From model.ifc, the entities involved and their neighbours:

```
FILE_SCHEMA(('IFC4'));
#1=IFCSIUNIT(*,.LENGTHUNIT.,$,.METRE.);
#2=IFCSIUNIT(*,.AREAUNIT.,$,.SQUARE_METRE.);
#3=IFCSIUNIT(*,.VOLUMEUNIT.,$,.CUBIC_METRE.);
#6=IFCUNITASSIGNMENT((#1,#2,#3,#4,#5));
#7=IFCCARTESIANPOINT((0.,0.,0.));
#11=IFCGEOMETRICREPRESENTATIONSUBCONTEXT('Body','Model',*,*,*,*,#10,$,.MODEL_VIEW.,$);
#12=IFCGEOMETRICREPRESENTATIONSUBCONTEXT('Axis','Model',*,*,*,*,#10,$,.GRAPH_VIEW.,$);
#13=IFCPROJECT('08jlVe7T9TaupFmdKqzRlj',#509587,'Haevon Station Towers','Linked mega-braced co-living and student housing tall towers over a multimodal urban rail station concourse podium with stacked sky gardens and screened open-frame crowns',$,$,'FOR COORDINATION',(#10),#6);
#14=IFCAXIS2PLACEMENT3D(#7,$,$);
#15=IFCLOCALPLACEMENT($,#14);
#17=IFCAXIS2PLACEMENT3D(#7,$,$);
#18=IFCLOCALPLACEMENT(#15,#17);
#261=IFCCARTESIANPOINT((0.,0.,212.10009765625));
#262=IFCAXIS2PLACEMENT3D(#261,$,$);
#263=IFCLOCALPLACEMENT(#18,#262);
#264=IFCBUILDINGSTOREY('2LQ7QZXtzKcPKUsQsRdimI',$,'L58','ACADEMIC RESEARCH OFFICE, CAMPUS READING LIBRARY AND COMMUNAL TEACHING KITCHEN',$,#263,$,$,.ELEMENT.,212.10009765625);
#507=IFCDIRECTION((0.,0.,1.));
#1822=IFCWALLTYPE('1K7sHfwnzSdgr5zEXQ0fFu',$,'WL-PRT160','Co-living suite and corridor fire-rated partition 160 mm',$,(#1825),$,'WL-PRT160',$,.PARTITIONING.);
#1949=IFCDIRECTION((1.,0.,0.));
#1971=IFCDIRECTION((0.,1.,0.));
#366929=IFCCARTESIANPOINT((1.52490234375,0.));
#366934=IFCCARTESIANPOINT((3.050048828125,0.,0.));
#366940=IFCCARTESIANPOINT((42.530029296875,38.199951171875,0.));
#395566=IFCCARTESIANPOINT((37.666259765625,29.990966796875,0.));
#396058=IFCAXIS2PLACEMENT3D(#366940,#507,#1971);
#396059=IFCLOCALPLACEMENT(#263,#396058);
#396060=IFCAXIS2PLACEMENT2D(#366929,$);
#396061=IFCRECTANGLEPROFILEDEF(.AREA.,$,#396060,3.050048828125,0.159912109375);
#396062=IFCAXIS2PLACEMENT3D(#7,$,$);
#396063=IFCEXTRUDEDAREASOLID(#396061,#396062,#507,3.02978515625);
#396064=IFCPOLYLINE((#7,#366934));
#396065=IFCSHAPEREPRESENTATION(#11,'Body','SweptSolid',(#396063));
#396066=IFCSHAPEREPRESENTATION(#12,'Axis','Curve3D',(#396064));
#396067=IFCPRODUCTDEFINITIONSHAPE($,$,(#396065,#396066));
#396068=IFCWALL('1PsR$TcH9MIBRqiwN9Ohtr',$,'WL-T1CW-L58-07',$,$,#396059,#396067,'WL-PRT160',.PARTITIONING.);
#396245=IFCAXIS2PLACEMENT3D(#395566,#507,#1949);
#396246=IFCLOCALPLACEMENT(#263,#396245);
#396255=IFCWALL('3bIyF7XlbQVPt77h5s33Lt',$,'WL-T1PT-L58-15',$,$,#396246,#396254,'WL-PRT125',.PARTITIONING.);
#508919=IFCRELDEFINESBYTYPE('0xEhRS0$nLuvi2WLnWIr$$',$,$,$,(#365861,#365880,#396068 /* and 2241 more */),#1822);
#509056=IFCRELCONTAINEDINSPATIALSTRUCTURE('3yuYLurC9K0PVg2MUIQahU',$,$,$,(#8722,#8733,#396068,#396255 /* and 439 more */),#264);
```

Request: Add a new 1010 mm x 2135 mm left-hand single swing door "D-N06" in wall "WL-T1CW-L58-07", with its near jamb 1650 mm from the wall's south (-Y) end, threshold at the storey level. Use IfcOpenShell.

```python
import numpy as np
import ifcopenshell
import ifcopenshell.api.feature
import ifcopenshell.api.geometry
import ifcopenshell.api.root
import ifcopenshell.api.spatial
import ifcopenshell.geom
import ifcopenshell.util.element
import ifcopenshell.util.placement
import ifcopenshell.util.representation
import ifcopenshell.util.shape
import ifcopenshell.util.unit

model = ifcopenshell.open("model.ifc")
unit_scale = ifcopenshell.util.unit.calculate_unit_scale(model)
settings = ifcopenshell.geom.settings()


def volume(element):
    """Net volume in cubic metres, openings subtracted."""
    shape = ifcopenshell.geom.create_shape(settings, element)
    return ifcopenshell.util.shape.get_volume(shape.geometry)


wall = model.by_guid("1PsR$TcH9MIBRqiwN9Ohtr")
storey = ifcopenshell.util.element.get_container(wall, ifc_class="IfcBuildingStorey")
context = ifcopenshell.util.representation.get_context(model, "Model", "Body", "MODEL_VIEW")
before = volume(wall)

width, height, from_end, sill = 1.01, 2.135, 1.65, 0.0  # metres

# The wall runs along its own X axis, and the end named is its -X end.
wall_shape = ifcopenshell.geom.create_shape(settings, wall)
x, y, z = ifcopenshell.util.shape.get_vertices(wall_shape.geometry).T
start = x.min() + from_end
face, thickness = float(y.min()), float(y.max() - y.min())
wall_matrix = ifcopenshell.util.placement.get_local_placement(wall.ObjectPlacement)
level = ifcopenshell.util.placement.get_local_placement(storey.ObjectPlacement)[2, 3]


def in_wall(x, y):
    """Placement at x, y metres in the wall's axes, at sill height."""
    matrix = wall_matrix.copy()
    matrix[:, 3] = wall_matrix @ np.array([x / unit_scale, y / unit_scale, 0.0, 1.0])
    matrix[2, 3] = level + sill / unit_scale
    return matrix


# Opening: a box that overshoots both wall faces by 50 mm.
opening = ifcopenshell.api.root.create_entity(model, ifc_class="IfcOpeningElement", predefined_type="OPENING")
box = ifcopenshell.api.geometry.add_wall_representation(
    model, context=context, length=width, height=height, thickness=thickness + 0.1
)
ifcopenshell.api.geometry.assign_representation(model, product=opening, representation=box)
ifcopenshell.api.geometry.edit_object_placement(model, product=opening, matrix=in_wall(start, face - 0.05), is_si=False)
ifcopenshell.api.feature.add_feature(model, feature=opening, element=wall)

door = ifcopenshell.api.root.create_entity(model, ifc_class="IfcDoor", name="D-N06", predefined_type="DOOR")
door.OverallWidth, door.OverallHeight = width / unit_scale, height / unit_scale
door.OperationType = "SINGLE_SWING_LEFT"
body = ifcopenshell.api.geometry.add_door_representation(
    model,
    context=context,
    overall_width=door.OverallWidth,
    overall_height=door.OverallHeight,
    operation_type="SINGLE_SWING_LEFT",
    lining_properties={"LiningDepth": thickness / unit_scale, "ThresholdDepth": thickness / unit_scale},
)
ifcopenshell.api.geometry.assign_representation(model, product=door, representation=body)
ifcopenshell.api.spatial.assign_container(model, products=[door], relating_structure=storey)
ifcopenshell.api.feature.add_filling(model, opening=opening, element=door)

# The lining spans the wall, so the door starts at the wall face.
ifcopenshell.api.geometry.edit_object_placement(model, product=door, matrix=in_wall(start, face), is_si=False)

after = volume(wall)

print(f"wall volume {before:.3f} -> {after:.3f} m3")

model.write("model_edited.ifc")
```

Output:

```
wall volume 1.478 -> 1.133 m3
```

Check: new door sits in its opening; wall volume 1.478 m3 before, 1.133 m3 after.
